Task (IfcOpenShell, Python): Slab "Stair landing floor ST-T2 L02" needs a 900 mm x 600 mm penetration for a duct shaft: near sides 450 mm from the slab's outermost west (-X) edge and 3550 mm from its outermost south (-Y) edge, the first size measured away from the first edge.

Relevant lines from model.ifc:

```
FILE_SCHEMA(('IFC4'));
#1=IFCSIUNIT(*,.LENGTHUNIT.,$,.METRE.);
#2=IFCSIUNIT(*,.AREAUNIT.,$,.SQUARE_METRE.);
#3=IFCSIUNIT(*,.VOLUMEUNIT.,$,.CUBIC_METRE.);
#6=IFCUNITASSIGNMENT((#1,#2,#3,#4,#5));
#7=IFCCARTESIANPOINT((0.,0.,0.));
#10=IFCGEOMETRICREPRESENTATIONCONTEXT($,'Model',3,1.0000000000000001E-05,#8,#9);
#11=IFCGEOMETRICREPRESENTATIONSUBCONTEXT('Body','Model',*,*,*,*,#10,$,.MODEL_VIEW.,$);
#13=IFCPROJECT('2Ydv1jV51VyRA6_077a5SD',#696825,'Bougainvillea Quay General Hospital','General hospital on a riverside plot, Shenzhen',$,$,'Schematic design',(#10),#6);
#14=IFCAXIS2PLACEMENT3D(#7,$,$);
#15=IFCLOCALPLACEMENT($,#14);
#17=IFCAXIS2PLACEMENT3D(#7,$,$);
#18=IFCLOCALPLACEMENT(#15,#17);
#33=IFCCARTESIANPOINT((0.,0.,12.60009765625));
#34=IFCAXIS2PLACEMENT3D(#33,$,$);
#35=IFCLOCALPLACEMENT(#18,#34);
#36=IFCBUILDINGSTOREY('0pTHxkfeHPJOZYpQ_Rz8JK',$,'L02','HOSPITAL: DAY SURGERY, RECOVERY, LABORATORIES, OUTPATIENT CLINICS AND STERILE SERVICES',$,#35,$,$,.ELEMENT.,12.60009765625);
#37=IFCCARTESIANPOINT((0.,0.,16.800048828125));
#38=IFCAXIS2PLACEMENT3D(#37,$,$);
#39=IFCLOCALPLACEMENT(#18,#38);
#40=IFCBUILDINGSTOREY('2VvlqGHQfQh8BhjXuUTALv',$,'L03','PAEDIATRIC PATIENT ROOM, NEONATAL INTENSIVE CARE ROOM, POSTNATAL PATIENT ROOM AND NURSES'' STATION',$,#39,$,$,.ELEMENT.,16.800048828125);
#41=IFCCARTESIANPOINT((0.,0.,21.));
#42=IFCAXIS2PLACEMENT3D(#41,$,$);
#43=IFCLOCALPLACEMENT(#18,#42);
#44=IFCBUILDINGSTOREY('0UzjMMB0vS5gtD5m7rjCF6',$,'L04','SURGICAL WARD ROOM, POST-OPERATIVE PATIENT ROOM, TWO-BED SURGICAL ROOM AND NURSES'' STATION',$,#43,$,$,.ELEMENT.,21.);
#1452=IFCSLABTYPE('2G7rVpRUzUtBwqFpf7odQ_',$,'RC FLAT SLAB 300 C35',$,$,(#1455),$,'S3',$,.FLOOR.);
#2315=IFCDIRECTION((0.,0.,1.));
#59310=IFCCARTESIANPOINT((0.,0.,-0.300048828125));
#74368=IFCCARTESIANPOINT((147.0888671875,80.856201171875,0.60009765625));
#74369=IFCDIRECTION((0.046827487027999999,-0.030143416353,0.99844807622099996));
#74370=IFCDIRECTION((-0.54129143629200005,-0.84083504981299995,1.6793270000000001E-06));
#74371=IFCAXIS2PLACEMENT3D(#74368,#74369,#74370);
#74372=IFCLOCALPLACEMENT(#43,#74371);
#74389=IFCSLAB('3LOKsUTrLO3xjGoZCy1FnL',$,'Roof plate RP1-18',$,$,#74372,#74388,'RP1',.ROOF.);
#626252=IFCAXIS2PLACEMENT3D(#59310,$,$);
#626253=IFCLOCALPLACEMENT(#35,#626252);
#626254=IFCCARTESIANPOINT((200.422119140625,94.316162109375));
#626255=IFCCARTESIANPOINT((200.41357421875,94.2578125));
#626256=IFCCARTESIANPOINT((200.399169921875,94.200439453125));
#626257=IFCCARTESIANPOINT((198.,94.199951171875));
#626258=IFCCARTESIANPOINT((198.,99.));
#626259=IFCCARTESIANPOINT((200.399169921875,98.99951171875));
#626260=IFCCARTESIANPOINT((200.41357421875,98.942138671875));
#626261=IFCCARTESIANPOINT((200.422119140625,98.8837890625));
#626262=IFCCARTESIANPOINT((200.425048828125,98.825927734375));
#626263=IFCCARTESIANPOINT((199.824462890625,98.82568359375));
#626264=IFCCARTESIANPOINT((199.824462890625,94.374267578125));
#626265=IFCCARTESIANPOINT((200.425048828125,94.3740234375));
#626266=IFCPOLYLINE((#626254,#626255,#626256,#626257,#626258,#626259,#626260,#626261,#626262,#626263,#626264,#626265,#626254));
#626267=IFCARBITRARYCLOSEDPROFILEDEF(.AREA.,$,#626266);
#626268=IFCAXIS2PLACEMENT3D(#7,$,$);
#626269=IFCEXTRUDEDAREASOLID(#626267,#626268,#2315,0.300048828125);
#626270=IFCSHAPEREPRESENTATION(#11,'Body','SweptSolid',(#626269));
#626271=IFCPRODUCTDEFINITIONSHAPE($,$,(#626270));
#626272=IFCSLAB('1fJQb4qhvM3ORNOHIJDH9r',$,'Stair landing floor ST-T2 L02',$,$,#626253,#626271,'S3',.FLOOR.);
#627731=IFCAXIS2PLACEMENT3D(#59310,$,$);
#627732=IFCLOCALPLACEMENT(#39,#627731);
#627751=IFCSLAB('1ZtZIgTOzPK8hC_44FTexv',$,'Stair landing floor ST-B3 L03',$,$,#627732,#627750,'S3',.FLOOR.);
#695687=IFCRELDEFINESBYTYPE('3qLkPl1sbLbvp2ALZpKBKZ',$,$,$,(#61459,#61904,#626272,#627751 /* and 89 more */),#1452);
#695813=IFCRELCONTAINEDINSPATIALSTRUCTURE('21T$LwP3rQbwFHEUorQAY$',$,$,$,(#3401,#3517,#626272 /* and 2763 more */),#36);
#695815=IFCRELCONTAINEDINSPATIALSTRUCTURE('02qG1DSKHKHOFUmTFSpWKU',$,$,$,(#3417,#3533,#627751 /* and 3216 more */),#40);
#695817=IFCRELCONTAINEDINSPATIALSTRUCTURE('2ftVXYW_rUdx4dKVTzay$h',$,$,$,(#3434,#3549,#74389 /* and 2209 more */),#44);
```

```python
import numpy as np
import ifcopenshell
import ifcopenshell.api.feature
import ifcopenshell.api.geometry
import ifcopenshell.api.root
import ifcopenshell.geom
import ifcopenshell.util.placement
import ifcopenshell.util.representation
import ifcopenshell.util.shape
import ifcopenshell.util.unit

model = ifcopenshell.open("model.ifc")
unit_scale = ifcopenshell.util.unit.calculate_unit_scale(model)
settings = ifcopenshell.geom.settings()


def volume(element):
    """Net volume in cubic metres, openings subtracted."""
    shape = ifcopenshell.geom.create_shape(settings, element)
    return ifcopenshell.util.shape.get_volume(shape.geometry)


slab = model.by_guid("1fJQb4qhvM3ORNOHIJDH9r")
before = volume(slab)

# Extent in the slab's own axes, in metres. The edges named are its -X and -Y sides.
slab_shape = ifcopenshell.geom.create_shape(settings, slab)
vertices = ifcopenshell.util.shape.get_vertices(slab_shape.geometry)
x_min, y_min, bottom = vertices.min(axis=0)
top = vertices[:, 2].max()

opening = ifcopenshell.api.root.create_entity(model, ifc_class="IfcOpeningElement", name="Duct shaft opening", predefined_type="OPENING")
context = ifcopenshell.util.representation.get_context(model, "Model", "Body", "MODEL_VIEW")
width, depth = 0.9, 0.6
outline = [(0.0, 0.0), (width, 0.0), (width, depth), (0.0, depth), (0.0, 0.0)]
# Overshoot both faces by 50 mm so the cut is clean.
shape = ifcopenshell.api.geometry.add_slab_representation(
    model, context=context, depth=top - bottom + 0.1, polyline=outline
)
ifcopenshell.api.geometry.assign_representation(model, product=opening, representation=shape)

matrix = ifcopenshell.util.placement.get_local_placement(slab.ObjectPlacement)
matrix[:, 3] = matrix @ np.append(np.array([x_min + 0.45, y_min + 3.55, bottom - 0.05]) / unit_scale, 1.0)
ifcopenshell.api.geometry.edit_object_placement(model, product=opening, matrix=matrix, is_si=False)
ifcopenshell.api.feature.add_feature(model, feature=opening, element=slab)

after = volume(slab)

print(f"slab volume {before:.3f} -> {after:.3f} m3")

model.write("model_rev.ifc")
```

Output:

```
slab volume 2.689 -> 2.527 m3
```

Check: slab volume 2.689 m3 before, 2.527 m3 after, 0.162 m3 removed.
